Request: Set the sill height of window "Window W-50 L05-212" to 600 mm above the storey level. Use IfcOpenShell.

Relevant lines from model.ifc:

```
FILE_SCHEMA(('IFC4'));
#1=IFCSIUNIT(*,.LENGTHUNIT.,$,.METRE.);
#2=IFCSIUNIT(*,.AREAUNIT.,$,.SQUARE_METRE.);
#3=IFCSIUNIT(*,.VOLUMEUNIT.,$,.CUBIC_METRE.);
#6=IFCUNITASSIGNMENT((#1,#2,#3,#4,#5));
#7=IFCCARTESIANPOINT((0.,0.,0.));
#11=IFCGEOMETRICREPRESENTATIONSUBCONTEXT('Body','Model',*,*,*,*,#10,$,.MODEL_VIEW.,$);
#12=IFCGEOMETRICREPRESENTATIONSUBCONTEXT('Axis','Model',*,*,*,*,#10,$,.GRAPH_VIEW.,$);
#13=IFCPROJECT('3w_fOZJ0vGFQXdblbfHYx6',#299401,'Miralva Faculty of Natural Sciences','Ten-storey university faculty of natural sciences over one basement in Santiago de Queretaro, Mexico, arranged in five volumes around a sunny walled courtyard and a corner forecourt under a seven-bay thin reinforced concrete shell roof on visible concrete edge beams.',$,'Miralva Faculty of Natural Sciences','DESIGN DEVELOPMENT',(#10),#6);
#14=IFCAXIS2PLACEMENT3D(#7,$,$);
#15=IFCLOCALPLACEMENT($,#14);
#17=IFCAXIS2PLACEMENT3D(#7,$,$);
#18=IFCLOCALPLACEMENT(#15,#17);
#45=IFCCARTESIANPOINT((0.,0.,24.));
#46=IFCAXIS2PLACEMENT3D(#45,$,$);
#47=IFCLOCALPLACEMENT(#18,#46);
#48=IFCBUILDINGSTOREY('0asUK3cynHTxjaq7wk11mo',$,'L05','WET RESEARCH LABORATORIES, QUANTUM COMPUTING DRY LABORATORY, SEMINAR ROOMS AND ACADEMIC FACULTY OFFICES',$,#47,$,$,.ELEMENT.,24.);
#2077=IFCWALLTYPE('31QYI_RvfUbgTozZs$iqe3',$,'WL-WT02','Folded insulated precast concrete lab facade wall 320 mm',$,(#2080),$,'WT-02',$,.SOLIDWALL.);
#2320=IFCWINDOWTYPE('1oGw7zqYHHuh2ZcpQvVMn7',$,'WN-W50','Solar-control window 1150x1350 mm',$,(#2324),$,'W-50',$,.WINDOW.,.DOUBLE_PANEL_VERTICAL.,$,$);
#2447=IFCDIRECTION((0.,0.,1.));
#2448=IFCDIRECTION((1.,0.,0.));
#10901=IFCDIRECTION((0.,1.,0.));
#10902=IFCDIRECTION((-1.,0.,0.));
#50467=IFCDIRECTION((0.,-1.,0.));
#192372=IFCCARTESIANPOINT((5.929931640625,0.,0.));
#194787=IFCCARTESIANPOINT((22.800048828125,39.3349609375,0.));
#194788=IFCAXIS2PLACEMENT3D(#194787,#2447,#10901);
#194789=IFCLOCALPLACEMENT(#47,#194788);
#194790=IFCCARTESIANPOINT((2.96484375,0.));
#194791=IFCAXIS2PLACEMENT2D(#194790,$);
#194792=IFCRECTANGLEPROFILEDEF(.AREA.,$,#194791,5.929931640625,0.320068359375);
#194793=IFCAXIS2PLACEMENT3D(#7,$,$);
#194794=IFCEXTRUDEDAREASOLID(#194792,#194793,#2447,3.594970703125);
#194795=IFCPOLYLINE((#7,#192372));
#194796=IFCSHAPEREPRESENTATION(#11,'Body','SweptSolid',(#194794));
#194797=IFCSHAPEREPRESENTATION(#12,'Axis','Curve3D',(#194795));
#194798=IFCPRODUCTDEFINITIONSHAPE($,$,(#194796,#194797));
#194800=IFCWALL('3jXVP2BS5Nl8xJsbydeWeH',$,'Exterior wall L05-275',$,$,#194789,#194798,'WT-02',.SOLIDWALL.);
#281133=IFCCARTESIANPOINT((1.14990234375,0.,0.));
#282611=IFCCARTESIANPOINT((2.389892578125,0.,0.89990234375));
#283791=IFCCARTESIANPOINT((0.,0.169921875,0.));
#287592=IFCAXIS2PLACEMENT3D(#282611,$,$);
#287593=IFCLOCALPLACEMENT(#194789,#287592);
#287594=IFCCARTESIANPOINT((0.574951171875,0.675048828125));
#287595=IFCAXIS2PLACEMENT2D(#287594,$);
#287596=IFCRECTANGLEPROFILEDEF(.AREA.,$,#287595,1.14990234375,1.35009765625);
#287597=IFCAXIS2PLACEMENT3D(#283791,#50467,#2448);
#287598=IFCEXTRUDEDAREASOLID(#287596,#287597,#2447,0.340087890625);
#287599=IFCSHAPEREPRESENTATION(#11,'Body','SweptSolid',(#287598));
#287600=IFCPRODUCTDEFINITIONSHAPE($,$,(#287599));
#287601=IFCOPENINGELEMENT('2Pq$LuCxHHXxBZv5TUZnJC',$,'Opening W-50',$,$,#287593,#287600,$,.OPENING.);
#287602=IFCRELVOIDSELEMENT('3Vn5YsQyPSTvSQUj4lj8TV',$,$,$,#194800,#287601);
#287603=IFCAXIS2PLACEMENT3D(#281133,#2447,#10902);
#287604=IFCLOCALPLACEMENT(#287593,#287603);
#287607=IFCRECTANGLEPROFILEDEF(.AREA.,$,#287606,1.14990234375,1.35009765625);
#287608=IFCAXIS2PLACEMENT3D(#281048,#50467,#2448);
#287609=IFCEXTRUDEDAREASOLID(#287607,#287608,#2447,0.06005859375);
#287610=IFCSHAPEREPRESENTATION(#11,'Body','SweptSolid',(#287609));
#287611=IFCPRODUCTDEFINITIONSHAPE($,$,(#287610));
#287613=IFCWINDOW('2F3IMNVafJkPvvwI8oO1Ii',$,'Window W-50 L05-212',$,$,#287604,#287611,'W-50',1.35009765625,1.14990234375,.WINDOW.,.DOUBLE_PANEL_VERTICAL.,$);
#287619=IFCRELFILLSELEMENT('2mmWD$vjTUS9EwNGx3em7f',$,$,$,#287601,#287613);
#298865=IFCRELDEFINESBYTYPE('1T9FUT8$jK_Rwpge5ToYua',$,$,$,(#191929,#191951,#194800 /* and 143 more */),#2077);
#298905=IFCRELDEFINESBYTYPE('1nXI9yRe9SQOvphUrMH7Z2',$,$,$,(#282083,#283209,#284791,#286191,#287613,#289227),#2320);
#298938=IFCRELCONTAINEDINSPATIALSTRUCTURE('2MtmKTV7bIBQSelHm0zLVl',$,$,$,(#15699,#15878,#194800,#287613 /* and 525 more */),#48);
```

```python
import numpy as np
import ifcopenshell
import ifcopenshell.api.geometry
import ifcopenshell.geom
import ifcopenshell.util.element
import ifcopenshell.util.placement
import ifcopenshell.util.shape
import ifcopenshell.util.unit

model = ifcopenshell.open("model.ifc")
unit_scale = ifcopenshell.util.unit.calculate_unit_scale(model)

window = model.by_id(287613)
opening = window.FillsVoids[0].RelatingOpeningElement
storey = ifcopenshell.util.element.get_container(window, ifc_class="IfcBuildingStorey")
level = ifcopenshell.util.placement.get_local_placement(storey.ObjectPlacement)[2, 3]

# The opening's origin need not be at the sill, so measure its lowest point.
shape = ifcopenshell.geom.create_shape(ifcopenshell.geom.settings(), opening)
bottom = ifcopenshell.util.shape.get_shape_bottom_elevation(shape, shape.geometry) / unit_scale
dz = level + 0.6 / unit_scale - bottom

shift = np.array([0.0, 0.0, dz])
# The window is placed relative to its opening, so it follows when the opening moves.
matrix = ifcopenshell.util.placement.get_local_placement(opening.ObjectPlacement)
matrix[:3, 3] += shift
ifcopenshell.api.geometry.edit_object_placement(
    model, product=opening, matrix=matrix, is_si=False, should_transform_children=True
)

print(f"moved by {dz * unit_scale:+.3f} m")

model.write("model_updated.ifc")
```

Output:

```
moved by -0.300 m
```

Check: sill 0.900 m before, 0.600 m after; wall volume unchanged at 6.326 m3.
